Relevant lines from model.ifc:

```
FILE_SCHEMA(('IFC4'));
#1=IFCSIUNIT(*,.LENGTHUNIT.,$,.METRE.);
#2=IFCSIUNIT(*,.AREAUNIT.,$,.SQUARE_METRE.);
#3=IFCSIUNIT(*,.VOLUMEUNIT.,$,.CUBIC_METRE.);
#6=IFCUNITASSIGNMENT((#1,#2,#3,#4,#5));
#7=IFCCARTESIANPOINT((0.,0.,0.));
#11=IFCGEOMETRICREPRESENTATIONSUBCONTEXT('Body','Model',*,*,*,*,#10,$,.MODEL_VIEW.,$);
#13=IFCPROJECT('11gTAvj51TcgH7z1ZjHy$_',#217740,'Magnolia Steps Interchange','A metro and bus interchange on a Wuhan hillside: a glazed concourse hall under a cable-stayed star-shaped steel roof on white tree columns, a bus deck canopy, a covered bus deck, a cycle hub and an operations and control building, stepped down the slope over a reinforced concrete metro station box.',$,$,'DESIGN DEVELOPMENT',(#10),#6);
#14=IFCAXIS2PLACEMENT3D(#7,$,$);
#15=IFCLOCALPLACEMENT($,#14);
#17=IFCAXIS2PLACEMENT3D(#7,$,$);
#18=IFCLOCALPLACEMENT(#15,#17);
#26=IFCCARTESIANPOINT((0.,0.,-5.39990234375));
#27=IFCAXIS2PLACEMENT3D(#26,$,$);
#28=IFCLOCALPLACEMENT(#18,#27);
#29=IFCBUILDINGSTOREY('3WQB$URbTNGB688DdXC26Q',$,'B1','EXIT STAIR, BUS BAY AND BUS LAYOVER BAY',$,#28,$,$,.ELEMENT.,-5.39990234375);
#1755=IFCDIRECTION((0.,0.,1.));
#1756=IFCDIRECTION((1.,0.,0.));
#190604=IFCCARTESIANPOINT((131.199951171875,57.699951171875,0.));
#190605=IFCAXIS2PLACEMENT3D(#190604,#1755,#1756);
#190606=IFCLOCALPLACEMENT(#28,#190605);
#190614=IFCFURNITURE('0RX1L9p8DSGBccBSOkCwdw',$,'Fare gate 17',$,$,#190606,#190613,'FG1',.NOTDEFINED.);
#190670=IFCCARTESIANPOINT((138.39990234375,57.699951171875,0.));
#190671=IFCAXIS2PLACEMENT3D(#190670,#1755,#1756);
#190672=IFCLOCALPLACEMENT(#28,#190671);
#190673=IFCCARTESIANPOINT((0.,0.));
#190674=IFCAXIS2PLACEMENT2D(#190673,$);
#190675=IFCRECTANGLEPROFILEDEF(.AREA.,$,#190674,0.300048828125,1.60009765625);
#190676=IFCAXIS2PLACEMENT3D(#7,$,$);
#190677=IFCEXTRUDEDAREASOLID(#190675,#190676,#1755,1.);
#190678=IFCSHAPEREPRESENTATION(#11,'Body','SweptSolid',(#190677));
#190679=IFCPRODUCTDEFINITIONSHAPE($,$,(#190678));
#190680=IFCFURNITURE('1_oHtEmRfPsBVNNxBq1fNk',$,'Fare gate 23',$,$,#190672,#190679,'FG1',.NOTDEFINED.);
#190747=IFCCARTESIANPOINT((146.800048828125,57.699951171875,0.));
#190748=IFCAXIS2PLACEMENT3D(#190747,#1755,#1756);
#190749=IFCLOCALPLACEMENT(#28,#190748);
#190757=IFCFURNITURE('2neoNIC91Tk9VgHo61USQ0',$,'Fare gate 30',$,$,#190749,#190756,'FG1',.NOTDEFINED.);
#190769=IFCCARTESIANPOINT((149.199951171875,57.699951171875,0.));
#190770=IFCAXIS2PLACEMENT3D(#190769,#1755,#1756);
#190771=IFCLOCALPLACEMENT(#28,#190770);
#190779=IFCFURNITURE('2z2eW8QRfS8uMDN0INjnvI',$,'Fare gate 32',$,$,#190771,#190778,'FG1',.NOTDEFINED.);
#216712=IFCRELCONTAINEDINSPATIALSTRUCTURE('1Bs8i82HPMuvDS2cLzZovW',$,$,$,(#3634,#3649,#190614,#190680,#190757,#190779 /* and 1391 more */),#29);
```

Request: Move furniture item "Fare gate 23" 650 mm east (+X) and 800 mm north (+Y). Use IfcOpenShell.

```python
import ifcopenshell
import ifcopenshell.api.geometry
import ifcopenshell.util.placement
import ifcopenshell.util.unit

model = ifcopenshell.open("model.ifc")
unit_scale = ifcopenshell.util.unit.calculate_unit_scale(model)

item = model.by_id(190680)
matrix = ifcopenshell.util.placement.get_local_placement(item.ObjectPlacement)
matrix[0, 3] += 0.65 / unit_scale
matrix[1, 3] += 0.8 / unit_scale
ifcopenshell.api.geometry.edit_object_placement(model, product=item, matrix=matrix, is_si=False)

print(ifcopenshell.util.placement.get_local_placement(item.ObjectPlacement).round(3) + 0.0)

model.write("model_edited.ifc")
```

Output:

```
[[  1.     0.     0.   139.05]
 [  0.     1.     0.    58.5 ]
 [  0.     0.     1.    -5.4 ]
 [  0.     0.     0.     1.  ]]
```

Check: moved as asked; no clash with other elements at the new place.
